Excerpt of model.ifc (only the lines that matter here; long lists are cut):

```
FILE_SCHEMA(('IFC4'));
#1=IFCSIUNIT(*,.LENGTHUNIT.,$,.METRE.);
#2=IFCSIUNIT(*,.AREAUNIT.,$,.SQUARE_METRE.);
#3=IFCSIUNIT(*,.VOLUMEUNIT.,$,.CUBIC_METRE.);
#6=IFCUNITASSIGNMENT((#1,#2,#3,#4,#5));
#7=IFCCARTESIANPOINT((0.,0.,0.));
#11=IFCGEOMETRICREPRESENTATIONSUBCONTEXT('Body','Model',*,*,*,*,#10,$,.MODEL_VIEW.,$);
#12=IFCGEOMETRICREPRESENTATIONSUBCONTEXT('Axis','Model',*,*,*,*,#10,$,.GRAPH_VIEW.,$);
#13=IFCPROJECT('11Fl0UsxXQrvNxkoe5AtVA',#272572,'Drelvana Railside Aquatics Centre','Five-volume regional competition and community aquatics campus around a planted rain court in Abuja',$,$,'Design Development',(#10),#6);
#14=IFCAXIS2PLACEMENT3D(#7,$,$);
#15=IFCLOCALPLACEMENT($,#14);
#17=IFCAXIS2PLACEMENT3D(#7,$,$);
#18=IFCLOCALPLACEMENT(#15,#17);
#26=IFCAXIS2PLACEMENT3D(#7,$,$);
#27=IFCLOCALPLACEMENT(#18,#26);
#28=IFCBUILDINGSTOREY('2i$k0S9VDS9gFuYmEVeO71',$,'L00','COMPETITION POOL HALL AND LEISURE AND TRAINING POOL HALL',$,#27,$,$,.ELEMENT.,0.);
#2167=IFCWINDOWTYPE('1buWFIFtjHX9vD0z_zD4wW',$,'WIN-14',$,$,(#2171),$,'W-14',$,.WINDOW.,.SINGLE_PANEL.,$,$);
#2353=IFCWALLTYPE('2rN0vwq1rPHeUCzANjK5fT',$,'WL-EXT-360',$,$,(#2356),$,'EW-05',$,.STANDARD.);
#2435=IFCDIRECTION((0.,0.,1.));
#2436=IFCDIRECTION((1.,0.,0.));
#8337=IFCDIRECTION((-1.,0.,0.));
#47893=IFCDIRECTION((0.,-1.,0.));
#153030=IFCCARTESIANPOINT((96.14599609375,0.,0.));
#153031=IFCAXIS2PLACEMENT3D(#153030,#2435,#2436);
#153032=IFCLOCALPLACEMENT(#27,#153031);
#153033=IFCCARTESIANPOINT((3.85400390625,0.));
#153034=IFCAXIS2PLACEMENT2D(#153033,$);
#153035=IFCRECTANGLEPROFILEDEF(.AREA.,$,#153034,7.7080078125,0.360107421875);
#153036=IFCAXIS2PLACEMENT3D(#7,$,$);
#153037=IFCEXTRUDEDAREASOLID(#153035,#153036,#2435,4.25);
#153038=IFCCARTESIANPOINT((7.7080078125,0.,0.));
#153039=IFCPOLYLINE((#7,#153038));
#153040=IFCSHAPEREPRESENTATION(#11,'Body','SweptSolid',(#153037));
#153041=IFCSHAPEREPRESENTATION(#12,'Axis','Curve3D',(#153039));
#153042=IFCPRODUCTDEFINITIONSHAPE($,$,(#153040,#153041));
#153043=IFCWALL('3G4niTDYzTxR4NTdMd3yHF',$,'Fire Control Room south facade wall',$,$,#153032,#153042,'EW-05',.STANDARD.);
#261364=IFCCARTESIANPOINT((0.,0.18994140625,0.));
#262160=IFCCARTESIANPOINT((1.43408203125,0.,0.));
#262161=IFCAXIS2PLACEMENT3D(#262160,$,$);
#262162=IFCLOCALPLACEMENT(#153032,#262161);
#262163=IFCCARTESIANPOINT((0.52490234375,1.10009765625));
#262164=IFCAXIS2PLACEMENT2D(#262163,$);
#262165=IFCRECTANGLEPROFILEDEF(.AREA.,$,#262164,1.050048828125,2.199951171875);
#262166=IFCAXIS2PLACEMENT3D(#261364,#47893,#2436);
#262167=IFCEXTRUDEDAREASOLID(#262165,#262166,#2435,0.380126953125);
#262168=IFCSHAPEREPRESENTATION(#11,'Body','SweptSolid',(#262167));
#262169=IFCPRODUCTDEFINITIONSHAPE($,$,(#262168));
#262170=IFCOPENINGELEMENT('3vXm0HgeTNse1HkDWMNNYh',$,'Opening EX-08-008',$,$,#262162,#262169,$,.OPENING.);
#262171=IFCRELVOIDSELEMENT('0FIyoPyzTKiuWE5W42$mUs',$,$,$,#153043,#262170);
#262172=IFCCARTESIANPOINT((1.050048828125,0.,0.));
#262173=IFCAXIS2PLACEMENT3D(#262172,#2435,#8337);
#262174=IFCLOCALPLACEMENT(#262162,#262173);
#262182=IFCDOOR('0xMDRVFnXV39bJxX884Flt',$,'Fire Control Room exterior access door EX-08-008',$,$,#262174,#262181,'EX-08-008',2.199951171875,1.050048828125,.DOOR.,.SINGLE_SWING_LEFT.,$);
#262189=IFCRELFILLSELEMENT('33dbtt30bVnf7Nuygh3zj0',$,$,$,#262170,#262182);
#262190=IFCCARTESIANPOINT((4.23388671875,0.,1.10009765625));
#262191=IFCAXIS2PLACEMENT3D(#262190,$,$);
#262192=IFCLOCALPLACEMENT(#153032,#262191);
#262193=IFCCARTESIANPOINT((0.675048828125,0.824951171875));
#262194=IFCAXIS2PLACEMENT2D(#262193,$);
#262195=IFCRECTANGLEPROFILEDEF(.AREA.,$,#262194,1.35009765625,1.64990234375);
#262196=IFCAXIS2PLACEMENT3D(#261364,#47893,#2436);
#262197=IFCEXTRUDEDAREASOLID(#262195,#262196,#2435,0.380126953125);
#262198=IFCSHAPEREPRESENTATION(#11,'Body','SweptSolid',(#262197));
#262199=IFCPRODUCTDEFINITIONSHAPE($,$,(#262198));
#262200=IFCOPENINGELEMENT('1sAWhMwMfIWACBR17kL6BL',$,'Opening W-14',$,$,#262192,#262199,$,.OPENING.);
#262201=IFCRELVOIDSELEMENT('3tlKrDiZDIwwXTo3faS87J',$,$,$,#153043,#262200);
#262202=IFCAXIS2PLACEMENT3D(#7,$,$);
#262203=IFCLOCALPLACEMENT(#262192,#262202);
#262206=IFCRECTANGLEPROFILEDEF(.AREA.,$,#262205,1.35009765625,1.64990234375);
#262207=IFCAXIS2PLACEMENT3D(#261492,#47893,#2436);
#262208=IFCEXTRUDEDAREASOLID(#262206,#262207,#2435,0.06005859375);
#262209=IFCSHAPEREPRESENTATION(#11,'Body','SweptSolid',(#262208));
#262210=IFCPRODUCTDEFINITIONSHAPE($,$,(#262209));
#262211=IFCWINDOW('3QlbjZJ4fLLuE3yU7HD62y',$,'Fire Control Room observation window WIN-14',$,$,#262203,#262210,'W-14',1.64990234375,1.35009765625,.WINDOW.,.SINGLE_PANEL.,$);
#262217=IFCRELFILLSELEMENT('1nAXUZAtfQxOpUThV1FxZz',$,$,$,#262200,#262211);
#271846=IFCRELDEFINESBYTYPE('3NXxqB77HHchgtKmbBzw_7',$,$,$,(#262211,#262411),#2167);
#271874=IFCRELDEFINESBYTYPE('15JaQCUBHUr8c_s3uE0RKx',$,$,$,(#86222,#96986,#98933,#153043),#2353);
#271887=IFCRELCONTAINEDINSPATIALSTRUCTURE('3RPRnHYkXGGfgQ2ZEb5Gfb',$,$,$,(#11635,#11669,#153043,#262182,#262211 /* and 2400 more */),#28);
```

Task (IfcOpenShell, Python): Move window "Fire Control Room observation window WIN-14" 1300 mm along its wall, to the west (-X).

```python
import ifcopenshell
import ifcopenshell.api.geometry
import ifcopenshell.util.placement

model = ifcopenshell.open("model.ifc")

window = model.by_guid("3QlbjZJ4fLLuE3yU7HD62y")
opening = window.FillsVoids[0].RelatingOpeningElement
wall = opening.VoidsElements[0].RelatingBuildingElement

wall_matrix = ifcopenshell.util.placement.get_local_placement(wall.ObjectPlacement)
shift = wall_matrix[:3, 0] * -1.3
before = ifcopenshell.util.placement.get_local_placement(window.ObjectPlacement)[:3, 3].copy()

# The window is placed relative to its opening, so it follows when the opening moves.
matrix = ifcopenshell.util.placement.get_local_placement(opening.ObjectPlacement)
matrix[:3, 3] += shift
ifcopenshell.api.geometry.edit_object_placement(
    model, product=opening, matrix=matrix, is_si=False, should_transform_children=True
)

after = ifcopenshell.util.placement.get_local_placement(window.ObjectPlacement)[:3, 3]
print("window moved by", (after - before).round(3) + 0.0)

model.write("model-out.ifc")
```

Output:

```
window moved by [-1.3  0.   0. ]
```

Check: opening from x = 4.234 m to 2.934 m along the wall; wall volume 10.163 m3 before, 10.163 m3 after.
